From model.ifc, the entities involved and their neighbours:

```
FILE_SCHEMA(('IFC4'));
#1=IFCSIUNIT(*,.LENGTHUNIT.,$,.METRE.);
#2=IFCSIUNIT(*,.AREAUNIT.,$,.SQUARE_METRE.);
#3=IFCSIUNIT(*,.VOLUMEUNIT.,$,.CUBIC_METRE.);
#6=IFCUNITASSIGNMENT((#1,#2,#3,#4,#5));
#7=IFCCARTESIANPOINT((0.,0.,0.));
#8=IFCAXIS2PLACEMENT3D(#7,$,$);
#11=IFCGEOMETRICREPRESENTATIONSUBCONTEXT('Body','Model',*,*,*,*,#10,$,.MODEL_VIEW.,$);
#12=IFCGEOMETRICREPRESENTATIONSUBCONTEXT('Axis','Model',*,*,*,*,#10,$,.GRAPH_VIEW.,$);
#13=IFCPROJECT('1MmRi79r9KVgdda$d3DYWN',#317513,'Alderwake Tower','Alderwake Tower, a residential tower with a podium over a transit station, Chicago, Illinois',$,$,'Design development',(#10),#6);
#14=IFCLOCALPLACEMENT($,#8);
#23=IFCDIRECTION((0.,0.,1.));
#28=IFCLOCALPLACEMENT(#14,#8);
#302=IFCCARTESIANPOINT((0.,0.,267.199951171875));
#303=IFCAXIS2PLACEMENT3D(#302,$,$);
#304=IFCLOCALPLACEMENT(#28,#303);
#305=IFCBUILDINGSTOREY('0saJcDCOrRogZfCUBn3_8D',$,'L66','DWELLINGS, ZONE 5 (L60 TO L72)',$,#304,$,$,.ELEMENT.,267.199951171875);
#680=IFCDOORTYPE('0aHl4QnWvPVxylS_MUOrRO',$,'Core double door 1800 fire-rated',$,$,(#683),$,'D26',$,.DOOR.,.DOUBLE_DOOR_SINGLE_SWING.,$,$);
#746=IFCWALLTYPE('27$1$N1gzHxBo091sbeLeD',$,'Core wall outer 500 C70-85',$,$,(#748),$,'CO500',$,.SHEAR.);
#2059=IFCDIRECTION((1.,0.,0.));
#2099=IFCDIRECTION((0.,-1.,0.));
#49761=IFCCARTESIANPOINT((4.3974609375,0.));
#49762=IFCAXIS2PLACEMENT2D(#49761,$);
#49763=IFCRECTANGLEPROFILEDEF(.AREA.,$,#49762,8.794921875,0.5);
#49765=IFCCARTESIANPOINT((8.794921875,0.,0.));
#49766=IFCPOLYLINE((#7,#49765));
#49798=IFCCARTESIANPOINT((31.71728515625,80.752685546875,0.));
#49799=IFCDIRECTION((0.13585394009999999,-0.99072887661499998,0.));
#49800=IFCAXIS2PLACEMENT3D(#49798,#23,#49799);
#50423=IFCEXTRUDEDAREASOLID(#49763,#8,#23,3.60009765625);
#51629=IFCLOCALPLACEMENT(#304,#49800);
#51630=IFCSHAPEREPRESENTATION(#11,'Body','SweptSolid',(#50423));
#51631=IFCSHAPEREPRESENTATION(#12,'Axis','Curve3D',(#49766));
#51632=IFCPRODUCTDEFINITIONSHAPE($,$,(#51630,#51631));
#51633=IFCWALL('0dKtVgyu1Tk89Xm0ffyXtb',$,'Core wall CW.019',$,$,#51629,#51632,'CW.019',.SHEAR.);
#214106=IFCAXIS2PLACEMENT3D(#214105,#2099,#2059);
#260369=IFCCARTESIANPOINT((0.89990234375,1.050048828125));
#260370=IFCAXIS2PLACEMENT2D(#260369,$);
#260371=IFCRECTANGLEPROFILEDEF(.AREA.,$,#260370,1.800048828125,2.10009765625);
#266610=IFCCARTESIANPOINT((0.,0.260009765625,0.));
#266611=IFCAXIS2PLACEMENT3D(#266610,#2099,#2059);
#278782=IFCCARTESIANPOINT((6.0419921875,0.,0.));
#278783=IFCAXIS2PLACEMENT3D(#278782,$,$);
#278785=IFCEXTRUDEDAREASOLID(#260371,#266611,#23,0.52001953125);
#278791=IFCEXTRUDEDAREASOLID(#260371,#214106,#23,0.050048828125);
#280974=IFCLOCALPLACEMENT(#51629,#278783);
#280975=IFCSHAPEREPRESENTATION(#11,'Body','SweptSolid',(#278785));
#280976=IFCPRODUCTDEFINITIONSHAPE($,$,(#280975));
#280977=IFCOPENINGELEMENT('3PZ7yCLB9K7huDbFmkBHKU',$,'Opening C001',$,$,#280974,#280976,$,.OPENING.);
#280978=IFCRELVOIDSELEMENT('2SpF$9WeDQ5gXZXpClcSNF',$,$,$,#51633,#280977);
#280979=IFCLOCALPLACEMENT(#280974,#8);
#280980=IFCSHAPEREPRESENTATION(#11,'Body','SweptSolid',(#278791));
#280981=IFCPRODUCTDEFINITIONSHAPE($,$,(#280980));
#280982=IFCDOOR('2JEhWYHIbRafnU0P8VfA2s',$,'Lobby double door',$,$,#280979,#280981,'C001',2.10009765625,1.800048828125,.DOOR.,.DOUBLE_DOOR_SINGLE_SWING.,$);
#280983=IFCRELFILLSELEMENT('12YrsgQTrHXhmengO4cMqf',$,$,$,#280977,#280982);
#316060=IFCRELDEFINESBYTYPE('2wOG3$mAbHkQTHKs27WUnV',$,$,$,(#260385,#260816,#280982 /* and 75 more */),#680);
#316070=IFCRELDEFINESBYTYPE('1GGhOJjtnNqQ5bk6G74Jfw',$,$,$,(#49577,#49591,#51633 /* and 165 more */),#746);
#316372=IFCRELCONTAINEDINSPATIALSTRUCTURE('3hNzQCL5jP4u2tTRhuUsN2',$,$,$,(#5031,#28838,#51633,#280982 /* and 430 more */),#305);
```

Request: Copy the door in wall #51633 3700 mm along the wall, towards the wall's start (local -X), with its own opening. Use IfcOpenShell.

```python
import ifcopenshell
import ifcopenshell.api.feature
import ifcopenshell.api.geometry
import ifcopenshell.api.root
import ifcopenshell.geom
import ifcopenshell.util.element
import ifcopenshell.util.placement
import ifcopenshell.util.shape
import ifcopenshell.util.unit

model = ifcopenshell.open("model.ifc")
unit_scale = ifcopenshell.util.unit.calculate_unit_scale(model)
settings = ifcopenshell.geom.settings()


def volume(element):
    """Net volume in cubic metres, openings subtracted."""
    shape = ifcopenshell.geom.create_shape(settings, element)
    return ifcopenshell.util.shape.get_volume(shape.geometry)


door = model.by_guid("2JEhWYHIbRafnU0P8VfA2s")
opening = door.FillsVoids[0].RelatingOpeningElement
wall = opening.VoidsElements[0].RelatingBuildingElement
before = volume(wall)
shift = ifcopenshell.util.placement.get_local_placement(wall.ObjectPlacement)[:3, 0] * -3.7 / unit_scale

# copy_class copies the void relationship, type, container and properties, but no geometry.
new_opening = ifcopenshell.api.root.copy_class(model, product=opening)
new_opening.Representation = ifcopenshell.util.element.copy_deep(
    model, opening.Representation, exclude=["IfcGeometricRepresentationContext", "IfcRepresentationMap"]
)
new_door = ifcopenshell.api.root.copy_class(model, product=door)
new_door.Representation = ifcopenshell.util.element.copy_deep(
    model, door.Representation, exclude=["IfcGeometricRepresentationContext", "IfcRepresentationMap"]
)
new_door.Tag = None
ifcopenshell.api.feature.add_filling(model, opening=new_opening, element=new_door)

for old, new in ((opening, new_opening), (door, new_door)):
    matrix = ifcopenshell.util.placement.get_local_placement(old.ObjectPlacement)
    matrix[:3, 3] += shift
    ifcopenshell.api.geometry.edit_object_placement(model, product=new, matrix=matrix, is_si=False)

after = volume(wall)

print(f"wall volume {before:.3f} -> {after:.3f} m3")

model.write("model-out.ifc")
```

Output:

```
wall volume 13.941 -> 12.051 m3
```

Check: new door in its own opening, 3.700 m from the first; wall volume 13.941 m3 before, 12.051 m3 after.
